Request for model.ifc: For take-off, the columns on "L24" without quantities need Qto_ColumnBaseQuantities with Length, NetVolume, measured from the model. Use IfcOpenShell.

First a look at what the model holds.

```python
import ifcopenshell
import ifcopenshell.util.element
import ifcopenshell.util.unit

model = ifcopenshell.open("model.ifc")
print(model.schema)
for unit_type in ("LENGTHUNIT", "AREAUNIT", "VOLUMEUNIT"):
    print(unit_type, ifcopenshell.util.unit.calculate_unit_scale(model, unit_type))
storey = next(s for s in model.by_type("IfcBuildingStorey") if s.Name == "L24")
columns = [e for e in ifcopenshell.util.element.get_decomposition(storey) if e.is_a("IfcColumn")]
for e in sorted(columns, key=lambda e: e.id()):
    print(e.id(), e.is_a(), e.Name, list(ifcopenshell.util.element.get_psets(e, qtos_only=True)), sep=" | ")
```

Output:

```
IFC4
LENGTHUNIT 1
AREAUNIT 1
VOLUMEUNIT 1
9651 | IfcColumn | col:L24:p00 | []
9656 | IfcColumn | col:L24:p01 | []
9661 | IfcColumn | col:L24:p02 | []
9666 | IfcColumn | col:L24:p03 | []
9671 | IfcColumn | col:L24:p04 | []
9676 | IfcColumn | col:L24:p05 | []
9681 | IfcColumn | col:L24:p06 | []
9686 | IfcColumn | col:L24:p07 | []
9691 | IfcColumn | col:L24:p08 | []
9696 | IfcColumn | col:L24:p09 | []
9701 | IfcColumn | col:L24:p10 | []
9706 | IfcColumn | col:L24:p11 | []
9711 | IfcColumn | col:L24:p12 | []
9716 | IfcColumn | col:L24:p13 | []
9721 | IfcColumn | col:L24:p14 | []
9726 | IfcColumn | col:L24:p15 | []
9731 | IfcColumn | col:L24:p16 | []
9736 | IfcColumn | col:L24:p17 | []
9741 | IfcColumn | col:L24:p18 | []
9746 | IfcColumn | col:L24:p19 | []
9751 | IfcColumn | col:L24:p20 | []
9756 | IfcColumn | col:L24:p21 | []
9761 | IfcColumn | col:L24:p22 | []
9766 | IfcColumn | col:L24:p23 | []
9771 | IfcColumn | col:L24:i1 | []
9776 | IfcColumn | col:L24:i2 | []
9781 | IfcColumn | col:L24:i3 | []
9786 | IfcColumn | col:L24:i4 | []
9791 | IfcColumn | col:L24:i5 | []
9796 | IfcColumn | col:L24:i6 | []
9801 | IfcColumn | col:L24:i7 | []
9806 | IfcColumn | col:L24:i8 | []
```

```python
import ifcopenshell
import ifcopenshell.api.pset
import ifcopenshell.geom
import ifcopenshell.util.element
import ifcopenshell.util.shape
import ifcopenshell.util.unit

model = ifcopenshell.open("model.ifc")
unit_scale = ifcopenshell.util.unit.calculate_unit_scale(model)
volume_scale = ifcopenshell.util.unit.calculate_unit_scale(model, "VOLUMEUNIT")
settings = ifcopenshell.geom.settings()

storey = next(s for s in model.by_type("IfcBuildingStorey") if s.Name == "L24")
columns = [e for e in ifcopenshell.util.element.get_decomposition(storey) if e.is_a("IfcColumn")]

for e in sorted(columns, key=lambda e: e.id()):
    if ifcopenshell.util.element.get_psets(e, qtos_only=True, should_inherit=False):
        continue
    # Geometry comes back in metres, in the element's own axes.
    shape = ifcopenshell.geom.create_shape(settings, e)
    values = {
        "Length": ifcopenshell.util.shape.get_z(shape.geometry) / unit_scale,
        "NetVolume": ifcopenshell.util.shape.get_volume(shape.geometry) / volume_scale,
    }
    qto = ifcopenshell.api.pset.add_qto(model, product=e, name="Qto_ColumnBaseQuantities")
    ifcopenshell.api.pset.edit_qto(model, qto=qto, properties=values)
    print(e.id(), {k: round(v, 3) for k, v in values.items()})

model.write("model-out.ifc")
```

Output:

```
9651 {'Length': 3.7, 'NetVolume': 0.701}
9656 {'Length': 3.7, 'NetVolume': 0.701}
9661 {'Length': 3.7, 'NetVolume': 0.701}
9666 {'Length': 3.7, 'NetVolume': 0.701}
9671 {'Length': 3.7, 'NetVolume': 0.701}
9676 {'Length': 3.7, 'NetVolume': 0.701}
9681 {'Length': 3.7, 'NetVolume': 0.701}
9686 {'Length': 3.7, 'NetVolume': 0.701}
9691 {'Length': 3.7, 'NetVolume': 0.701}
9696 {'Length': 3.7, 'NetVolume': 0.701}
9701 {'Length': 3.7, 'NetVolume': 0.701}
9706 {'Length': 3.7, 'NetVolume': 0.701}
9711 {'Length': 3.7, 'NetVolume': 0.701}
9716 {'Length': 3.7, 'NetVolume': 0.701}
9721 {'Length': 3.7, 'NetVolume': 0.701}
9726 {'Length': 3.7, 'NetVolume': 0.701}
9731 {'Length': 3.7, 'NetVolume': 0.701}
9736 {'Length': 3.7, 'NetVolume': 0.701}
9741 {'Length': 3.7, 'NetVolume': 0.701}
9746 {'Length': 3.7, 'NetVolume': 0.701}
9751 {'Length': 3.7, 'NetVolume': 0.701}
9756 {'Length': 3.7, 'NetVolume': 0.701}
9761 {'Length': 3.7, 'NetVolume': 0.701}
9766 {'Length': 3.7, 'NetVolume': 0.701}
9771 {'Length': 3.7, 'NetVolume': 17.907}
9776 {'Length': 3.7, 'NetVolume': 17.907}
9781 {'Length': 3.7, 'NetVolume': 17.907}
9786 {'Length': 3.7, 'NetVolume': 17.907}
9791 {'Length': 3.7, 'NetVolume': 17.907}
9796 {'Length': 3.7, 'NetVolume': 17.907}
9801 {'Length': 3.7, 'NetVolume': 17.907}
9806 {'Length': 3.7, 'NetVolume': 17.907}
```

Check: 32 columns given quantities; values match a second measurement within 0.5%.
